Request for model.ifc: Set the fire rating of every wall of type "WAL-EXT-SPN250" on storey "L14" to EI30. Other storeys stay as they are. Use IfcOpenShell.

First a look at what the model holds.

```python
import ifcopenshell
import ifcopenshell.util.element

model = ifcopenshell.open("model.ifc")
print(model.schema)
storey = next(s for s in model.by_type("IfcBuildingStorey") if s.Name == "L14")
walls = [e for e in ifcopenshell.util.element.get_decomposition(storey) if e.is_a("IfcWall")]
seen = {}
for e in walls:
    element_type = ifcopenshell.util.element.get_type(e)
    key = (element_type.Name if element_type != e and element_type else None, ifcopenshell.util.element.get_pset(e, "Pset_WallCommon", "FireRating"))
    seen[key] = seen.get(key, 0) + 1
for (name, value), count in sorted(seen.items(), key=str):
    print(count, "x", name, "|", value)
```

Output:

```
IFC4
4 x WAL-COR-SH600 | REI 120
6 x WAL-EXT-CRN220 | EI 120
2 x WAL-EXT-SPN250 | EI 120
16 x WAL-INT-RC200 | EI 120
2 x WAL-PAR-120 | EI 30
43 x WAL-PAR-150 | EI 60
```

```python
import ifcopenshell
import ifcopenshell.api.pset
import ifcopenshell.util.element

model = ifcopenshell.open("model.ifc")

storey = next(s for s in model.by_type("IfcBuildingStorey") if s.Name == "L14")
walls = [e for e in ifcopenshell.util.element.get_decomposition(storey) if e.is_a("IfcWall")]

count = 0
for e in walls:
    element_type = ifcopenshell.util.element.get_type(e)
    if element_type in (None, e) or element_type.Name != "WAL-EXT-SPN250":
        continue
    found = ifcopenshell.util.element.get_pset(e, "Pset_WallCommon", should_inherit=False)
    if found:
        pset = model.by_id(found["id"])
        if len(ifcopenshell.util.element.get_elements_by_pset(pset)) > 1:
            pset = ifcopenshell.api.pset.unshare_pset(model, products=[e], pset=pset)[0]
    else:
        pset = ifcopenshell.api.pset.add_pset(model, product=e, name="Pset_WallCommon")
    ifcopenshell.api.pset.edit_pset(model, pset=pset, properties={"FireRating": "EI30"})
    count += 1

print(count, "walls updated")

model.write("model_updated.ifc")
```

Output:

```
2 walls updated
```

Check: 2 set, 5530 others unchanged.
